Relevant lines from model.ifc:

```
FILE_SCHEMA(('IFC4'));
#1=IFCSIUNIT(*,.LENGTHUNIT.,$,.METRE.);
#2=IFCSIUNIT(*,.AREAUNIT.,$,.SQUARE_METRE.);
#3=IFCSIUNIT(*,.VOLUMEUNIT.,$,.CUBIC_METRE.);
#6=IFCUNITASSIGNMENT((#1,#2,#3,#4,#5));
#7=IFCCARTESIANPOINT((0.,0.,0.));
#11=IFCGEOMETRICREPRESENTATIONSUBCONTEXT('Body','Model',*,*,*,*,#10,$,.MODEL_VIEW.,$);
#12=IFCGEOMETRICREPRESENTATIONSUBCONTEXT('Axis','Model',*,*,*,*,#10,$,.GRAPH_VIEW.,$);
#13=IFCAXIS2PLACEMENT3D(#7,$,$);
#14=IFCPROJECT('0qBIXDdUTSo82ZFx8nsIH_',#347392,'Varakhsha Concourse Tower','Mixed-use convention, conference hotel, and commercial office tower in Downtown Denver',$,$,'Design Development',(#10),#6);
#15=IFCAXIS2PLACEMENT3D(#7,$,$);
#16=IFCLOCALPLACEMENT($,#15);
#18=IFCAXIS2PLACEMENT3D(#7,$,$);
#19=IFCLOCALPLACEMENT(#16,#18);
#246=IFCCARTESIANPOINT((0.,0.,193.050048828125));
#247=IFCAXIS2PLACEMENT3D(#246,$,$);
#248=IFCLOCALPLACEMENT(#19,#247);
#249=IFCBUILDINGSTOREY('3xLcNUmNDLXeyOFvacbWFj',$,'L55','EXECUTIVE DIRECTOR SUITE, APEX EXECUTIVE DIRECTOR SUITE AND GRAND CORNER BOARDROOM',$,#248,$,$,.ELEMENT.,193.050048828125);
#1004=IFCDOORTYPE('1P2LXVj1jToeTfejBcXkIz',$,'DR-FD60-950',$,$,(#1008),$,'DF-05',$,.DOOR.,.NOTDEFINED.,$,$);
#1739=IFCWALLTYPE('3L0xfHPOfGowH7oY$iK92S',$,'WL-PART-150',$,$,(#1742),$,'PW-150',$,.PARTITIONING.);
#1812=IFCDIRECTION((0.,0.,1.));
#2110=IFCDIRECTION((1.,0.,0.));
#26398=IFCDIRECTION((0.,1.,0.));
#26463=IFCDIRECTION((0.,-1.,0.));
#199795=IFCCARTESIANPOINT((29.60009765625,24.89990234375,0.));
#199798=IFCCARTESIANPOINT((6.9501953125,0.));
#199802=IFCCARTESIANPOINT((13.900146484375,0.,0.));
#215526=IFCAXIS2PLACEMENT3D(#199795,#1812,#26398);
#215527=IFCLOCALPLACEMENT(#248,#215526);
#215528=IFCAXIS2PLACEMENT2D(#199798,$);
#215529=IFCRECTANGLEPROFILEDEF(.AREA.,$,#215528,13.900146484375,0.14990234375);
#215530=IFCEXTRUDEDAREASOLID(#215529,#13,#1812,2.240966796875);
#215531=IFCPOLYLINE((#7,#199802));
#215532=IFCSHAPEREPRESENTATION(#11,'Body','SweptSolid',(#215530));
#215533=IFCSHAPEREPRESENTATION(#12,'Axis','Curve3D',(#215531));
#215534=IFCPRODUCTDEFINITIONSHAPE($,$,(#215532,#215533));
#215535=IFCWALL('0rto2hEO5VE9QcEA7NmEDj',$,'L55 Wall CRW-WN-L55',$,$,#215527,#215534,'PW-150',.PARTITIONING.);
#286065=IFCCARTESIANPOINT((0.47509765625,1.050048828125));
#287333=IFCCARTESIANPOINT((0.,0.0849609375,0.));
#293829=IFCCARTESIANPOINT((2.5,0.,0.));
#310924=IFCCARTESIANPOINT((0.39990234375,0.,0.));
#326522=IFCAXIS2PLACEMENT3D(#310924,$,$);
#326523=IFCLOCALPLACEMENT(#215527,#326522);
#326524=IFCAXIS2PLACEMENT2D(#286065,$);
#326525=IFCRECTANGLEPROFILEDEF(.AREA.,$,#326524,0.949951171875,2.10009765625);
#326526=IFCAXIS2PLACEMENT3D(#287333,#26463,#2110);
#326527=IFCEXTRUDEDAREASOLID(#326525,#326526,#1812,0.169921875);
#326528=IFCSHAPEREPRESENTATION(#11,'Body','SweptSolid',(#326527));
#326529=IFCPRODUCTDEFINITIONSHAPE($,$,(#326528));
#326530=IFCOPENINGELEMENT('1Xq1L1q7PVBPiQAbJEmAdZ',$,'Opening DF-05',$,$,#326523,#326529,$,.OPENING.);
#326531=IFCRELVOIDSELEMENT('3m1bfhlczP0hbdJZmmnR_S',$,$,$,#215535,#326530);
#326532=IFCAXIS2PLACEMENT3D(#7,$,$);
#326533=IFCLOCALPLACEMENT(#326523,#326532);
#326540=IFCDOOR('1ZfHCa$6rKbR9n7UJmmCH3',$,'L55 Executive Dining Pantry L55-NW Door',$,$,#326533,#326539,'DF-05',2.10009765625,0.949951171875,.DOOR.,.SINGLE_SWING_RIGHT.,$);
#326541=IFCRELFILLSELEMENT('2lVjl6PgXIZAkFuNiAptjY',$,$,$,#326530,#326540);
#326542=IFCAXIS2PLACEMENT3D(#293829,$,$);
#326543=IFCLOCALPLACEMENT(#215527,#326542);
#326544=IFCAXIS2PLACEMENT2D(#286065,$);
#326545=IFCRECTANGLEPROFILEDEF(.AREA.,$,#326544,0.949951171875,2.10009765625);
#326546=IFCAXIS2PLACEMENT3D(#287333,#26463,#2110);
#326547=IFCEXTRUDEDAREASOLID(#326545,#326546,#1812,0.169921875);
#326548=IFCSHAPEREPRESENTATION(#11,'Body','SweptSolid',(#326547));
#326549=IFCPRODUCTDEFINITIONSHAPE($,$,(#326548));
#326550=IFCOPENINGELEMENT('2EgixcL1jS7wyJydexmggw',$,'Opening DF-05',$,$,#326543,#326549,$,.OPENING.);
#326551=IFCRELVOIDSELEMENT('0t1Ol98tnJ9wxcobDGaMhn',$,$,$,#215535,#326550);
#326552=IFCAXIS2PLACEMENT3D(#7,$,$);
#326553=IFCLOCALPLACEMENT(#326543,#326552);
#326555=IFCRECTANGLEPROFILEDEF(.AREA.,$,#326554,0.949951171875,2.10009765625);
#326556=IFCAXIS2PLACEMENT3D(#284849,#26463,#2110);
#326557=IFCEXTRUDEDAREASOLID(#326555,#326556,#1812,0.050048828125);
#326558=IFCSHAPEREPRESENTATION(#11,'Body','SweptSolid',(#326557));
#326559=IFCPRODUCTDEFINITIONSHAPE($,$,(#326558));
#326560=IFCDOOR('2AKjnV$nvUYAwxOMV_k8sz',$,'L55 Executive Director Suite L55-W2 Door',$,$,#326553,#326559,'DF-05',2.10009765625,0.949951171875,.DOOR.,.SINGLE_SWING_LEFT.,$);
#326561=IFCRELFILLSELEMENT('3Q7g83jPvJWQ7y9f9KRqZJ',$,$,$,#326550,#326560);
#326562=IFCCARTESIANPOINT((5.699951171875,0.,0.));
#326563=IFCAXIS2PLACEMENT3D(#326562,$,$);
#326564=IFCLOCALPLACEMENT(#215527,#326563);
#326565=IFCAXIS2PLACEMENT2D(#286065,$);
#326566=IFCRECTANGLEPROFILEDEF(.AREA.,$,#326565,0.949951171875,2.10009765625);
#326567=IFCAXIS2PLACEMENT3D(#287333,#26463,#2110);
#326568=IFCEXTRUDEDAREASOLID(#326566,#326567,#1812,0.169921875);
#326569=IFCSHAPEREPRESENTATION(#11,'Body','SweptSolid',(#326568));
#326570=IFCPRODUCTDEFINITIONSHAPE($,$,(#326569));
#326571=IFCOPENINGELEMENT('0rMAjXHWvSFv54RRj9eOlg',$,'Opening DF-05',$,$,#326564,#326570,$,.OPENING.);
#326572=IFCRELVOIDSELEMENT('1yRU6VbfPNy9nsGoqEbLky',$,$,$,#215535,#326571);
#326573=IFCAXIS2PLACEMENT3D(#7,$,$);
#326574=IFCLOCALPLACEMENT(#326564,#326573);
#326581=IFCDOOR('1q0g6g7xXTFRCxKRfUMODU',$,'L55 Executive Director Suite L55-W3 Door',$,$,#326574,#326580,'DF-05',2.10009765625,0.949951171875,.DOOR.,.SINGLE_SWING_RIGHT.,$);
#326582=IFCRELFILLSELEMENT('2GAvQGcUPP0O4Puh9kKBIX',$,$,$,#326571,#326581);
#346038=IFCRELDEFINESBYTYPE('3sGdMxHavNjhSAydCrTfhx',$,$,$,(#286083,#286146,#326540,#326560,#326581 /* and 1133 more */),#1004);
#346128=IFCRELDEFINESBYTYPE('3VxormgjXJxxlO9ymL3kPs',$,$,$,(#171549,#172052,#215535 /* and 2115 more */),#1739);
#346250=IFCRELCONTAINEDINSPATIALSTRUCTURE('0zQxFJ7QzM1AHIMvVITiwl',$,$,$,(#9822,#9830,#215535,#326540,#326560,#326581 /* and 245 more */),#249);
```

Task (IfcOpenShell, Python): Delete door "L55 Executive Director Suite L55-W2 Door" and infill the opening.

```python
import ifcopenshell
import ifcopenshell.api.feature
import ifcopenshell.api.root
import ifcopenshell.geom
import ifcopenshell.util.shape

model = ifcopenshell.open("model.ifc")
settings = ifcopenshell.geom.settings()


def volume(element):
    """Net volume in cubic metres, openings subtracted."""
    shape = ifcopenshell.geom.create_shape(settings, element)
    return ifcopenshell.util.shape.get_volume(shape.geometry)


door = model.by_guid("2AKjnV$nvUYAwxOMV_k8sz")
opening = door.FillsVoids[0].RelatingOpeningElement
wall = opening.VoidsElements[0].RelatingBuildingElement
before = volume(wall)

ifcopenshell.api.root.remove_product(model, product=door)
ifcopenshell.api.feature.remove_feature(model, feature=opening)

after = volume(wall)

print(f"wall volume {before:.3f} -> {after:.3f} m3")

model.write("model_edited.ifc")
```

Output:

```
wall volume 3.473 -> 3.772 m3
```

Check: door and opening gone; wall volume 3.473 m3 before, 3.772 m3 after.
